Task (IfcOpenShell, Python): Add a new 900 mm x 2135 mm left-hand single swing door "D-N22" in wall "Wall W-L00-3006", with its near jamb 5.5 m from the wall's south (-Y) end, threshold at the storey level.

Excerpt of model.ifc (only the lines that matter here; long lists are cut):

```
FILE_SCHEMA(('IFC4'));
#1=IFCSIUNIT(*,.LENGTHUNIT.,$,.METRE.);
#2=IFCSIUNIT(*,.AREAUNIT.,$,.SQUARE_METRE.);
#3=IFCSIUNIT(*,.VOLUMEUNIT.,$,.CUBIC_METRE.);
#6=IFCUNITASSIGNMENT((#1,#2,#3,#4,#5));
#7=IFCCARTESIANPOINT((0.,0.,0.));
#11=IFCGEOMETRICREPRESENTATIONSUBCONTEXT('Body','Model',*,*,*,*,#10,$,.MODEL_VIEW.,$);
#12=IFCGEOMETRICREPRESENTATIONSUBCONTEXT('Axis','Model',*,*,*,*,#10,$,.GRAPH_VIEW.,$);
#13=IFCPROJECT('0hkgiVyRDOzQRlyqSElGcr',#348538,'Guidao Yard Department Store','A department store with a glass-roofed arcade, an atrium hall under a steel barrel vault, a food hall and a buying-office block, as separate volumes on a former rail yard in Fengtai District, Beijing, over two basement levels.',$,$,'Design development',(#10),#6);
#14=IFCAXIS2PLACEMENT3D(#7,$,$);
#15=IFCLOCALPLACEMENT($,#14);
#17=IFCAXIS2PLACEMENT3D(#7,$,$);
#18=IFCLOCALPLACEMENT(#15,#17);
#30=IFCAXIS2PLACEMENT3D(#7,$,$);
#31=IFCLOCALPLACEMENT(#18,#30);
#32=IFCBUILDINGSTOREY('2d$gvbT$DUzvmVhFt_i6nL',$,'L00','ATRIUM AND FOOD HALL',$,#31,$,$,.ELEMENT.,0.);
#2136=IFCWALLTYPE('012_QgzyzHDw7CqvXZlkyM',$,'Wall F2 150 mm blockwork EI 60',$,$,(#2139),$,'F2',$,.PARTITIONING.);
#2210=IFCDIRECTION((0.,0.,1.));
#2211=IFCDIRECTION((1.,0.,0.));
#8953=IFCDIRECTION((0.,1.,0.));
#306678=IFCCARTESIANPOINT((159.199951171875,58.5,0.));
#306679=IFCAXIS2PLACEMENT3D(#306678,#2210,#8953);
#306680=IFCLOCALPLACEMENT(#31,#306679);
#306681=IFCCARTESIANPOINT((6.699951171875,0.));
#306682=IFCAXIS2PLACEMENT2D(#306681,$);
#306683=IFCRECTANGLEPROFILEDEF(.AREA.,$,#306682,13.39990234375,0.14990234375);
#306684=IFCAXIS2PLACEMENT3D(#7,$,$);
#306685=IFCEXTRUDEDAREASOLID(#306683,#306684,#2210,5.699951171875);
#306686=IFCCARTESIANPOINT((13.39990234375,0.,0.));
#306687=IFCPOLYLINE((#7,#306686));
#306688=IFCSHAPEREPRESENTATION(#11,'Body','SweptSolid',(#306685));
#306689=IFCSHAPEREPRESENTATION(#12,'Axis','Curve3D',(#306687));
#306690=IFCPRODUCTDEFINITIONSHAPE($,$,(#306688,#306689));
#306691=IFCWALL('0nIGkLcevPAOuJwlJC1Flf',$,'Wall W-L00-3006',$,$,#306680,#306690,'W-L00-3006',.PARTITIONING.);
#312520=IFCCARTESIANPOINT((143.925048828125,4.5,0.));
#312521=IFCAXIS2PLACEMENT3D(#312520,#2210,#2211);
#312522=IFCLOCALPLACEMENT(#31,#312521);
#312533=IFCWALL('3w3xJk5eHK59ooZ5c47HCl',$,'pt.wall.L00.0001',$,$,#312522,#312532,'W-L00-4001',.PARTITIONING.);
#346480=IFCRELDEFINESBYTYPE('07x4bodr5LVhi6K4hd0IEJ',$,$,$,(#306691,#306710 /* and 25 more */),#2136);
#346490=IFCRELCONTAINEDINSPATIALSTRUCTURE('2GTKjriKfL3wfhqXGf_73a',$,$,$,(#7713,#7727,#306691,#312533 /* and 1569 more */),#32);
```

```python
import numpy as np
import ifcopenshell
import ifcopenshell.api.feature
import ifcopenshell.api.geometry
import ifcopenshell.api.root
import ifcopenshell.api.spatial
import ifcopenshell.geom
import ifcopenshell.util.element
import ifcopenshell.util.placement
import ifcopenshell.util.representation
import ifcopenshell.util.shape
import ifcopenshell.util.unit

model = ifcopenshell.open("model.ifc")
unit_scale = ifcopenshell.util.unit.calculate_unit_scale(model)
settings = ifcopenshell.geom.settings()


def volume(element):
    """Net volume in cubic metres, openings subtracted."""
    shape = ifcopenshell.geom.create_shape(settings, element)
    return ifcopenshell.util.shape.get_volume(shape.geometry)


wall = model.by_guid("0nIGkLcevPAOuJwlJC1Flf")
storey = ifcopenshell.util.element.get_container(wall, ifc_class="IfcBuildingStorey")
context = ifcopenshell.util.representation.get_context(model, "Model", "Body", "MODEL_VIEW")
before = volume(wall)

width, height, from_end, sill = 0.9, 2.135, 5.5, 0.0  # metres

# The wall runs along its own X axis, and the end named is its -X end.
wall_shape = ifcopenshell.geom.create_shape(settings, wall)
x, y, z = ifcopenshell.util.shape.get_vertices(wall_shape.geometry).T
start = x.min() + from_end
face, thickness = float(y.min()), float(y.max() - y.min())
wall_matrix = ifcopenshell.util.placement.get_local_placement(wall.ObjectPlacement)
level = ifcopenshell.util.placement.get_local_placement(storey.ObjectPlacement)[2, 3]


def in_wall(x, y):
    """Placement at x, y metres in the wall's axes, at sill height."""
    matrix = wall_matrix.copy()
    matrix[:, 3] = wall_matrix @ np.array([x / unit_scale, y / unit_scale, 0.0, 1.0])
    matrix[2, 3] = level + sill / unit_scale
    return matrix


# Opening: a box that overshoots both wall faces by 50 mm.
opening = ifcopenshell.api.root.create_entity(model, ifc_class="IfcOpeningElement", predefined_type="OPENING")
box = ifcopenshell.api.geometry.add_wall_representation(
    model, context=context, length=width, height=height, thickness=thickness + 0.1
)
ifcopenshell.api.geometry.assign_representation(model, product=opening, representation=box)
ifcopenshell.api.geometry.edit_object_placement(model, product=opening, matrix=in_wall(start, face - 0.05), is_si=False)
ifcopenshell.api.feature.add_feature(model, feature=opening, element=wall)

door = ifcopenshell.api.root.create_entity(model, ifc_class="IfcDoor", name="D-N22", predefined_type="DOOR")
door.OverallWidth, door.OverallHeight = width / unit_scale, height / unit_scale
door.OperationType = "SINGLE_SWING_LEFT"
body = ifcopenshell.api.geometry.add_door_representation(
    model,
    context=context,
    overall_width=door.OverallWidth,
    overall_height=door.OverallHeight,
    operation_type="SINGLE_SWING_LEFT",
    lining_properties={"LiningDepth": thickness / unit_scale, "ThresholdDepth": thickness / unit_scale},
)
ifcopenshell.api.geometry.assign_representation(model, product=door, representation=body)
ifcopenshell.api.spatial.assign_container(model, products=[door], relating_structure=storey)
ifcopenshell.api.feature.add_filling(model, opening=opening, element=door)

# The lining spans the wall, so the door starts at the wall face.
ifcopenshell.api.geometry.edit_object_placement(model, product=door, matrix=in_wall(start, face), is_si=False)

after = volume(wall)

print(f"wall volume {before:.3f} -> {after:.3f} m3")

model.write("model_updated.ifc")
```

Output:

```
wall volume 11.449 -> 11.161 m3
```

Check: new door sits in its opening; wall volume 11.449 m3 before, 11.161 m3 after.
